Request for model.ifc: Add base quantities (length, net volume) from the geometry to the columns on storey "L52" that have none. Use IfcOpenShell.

First a look at what the model holds.

```python
import ifcopenshell
import ifcopenshell.util.element
import ifcopenshell.util.unit

model = ifcopenshell.open("model.ifc")
print(model.schema)
for unit_type in ("LENGTHUNIT", "AREAUNIT", "VOLUMEUNIT"):
    print(unit_type, ifcopenshell.util.unit.calculate_unit_scale(model, unit_type))
storey = next(s for s in model.by_type("IfcBuildingStorey") if s.Name == "L52")
columns = [e for e in ifcopenshell.util.element.get_decomposition(storey) if e.is_a("IfcColumn")]
for e in sorted(columns, key=lambda e: e.id()):
    print(e.id(), e.is_a(), e.Name, list(ifcopenshell.util.element.get_psets(e, qtos_only=True)), sep=" | ")
```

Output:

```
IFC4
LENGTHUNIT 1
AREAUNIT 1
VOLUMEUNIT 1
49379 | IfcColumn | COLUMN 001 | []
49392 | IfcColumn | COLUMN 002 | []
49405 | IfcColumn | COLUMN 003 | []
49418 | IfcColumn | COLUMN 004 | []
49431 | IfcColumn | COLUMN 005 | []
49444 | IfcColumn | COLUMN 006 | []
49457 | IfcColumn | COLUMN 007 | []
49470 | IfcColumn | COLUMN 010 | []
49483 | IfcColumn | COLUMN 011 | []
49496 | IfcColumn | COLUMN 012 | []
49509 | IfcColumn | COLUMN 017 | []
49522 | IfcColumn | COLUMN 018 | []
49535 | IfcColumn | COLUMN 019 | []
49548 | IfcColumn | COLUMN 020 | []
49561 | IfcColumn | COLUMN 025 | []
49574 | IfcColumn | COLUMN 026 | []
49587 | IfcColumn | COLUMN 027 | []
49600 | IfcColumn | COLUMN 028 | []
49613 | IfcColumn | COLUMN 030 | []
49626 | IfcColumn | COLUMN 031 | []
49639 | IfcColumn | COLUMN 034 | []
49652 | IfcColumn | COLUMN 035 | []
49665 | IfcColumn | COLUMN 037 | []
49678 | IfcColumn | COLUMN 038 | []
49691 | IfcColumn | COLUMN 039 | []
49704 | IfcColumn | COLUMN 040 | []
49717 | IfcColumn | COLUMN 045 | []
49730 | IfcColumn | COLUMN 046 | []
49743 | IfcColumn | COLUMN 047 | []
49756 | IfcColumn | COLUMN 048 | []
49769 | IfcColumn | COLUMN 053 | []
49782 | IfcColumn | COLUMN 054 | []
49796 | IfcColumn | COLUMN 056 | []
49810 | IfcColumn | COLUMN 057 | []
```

```python
import ifcopenshell
import ifcopenshell.api.pset
import ifcopenshell.geom
import ifcopenshell.util.element
import ifcopenshell.util.shape
import ifcopenshell.util.unit

model = ifcopenshell.open("model.ifc")
unit_scale = ifcopenshell.util.unit.calculate_unit_scale(model)
volume_scale = ifcopenshell.util.unit.calculate_unit_scale(model, "VOLUMEUNIT")
settings = ifcopenshell.geom.settings()

storey = next(s for s in model.by_type("IfcBuildingStorey") if s.Name == "L52")
columns = [e for e in ifcopenshell.util.element.get_decomposition(storey) if e.is_a("IfcColumn")]

for e in sorted(columns, key=lambda e: e.id()):
    if ifcopenshell.util.element.get_psets(e, qtos_only=True, should_inherit=False):
        continue
    # Geometry comes back in metres, in the element's own axes.
    shape = ifcopenshell.geom.create_shape(settings, e)
    values = {
        "Length": ifcopenshell.util.shape.get_z(shape.geometry) / unit_scale,
        "NetVolume": ifcopenshell.util.shape.get_volume(shape.geometry) / volume_scale,
    }
    qto = ifcopenshell.api.pset.add_qto(model, product=e, name="Qto_ColumnBaseQuantities")
    ifcopenshell.api.pset.edit_qto(model, qto=qto, properties=values)
    print(e.id(), {k: round(v, 3) for k, v in values.items()})

model.write("model-out.ifc")
```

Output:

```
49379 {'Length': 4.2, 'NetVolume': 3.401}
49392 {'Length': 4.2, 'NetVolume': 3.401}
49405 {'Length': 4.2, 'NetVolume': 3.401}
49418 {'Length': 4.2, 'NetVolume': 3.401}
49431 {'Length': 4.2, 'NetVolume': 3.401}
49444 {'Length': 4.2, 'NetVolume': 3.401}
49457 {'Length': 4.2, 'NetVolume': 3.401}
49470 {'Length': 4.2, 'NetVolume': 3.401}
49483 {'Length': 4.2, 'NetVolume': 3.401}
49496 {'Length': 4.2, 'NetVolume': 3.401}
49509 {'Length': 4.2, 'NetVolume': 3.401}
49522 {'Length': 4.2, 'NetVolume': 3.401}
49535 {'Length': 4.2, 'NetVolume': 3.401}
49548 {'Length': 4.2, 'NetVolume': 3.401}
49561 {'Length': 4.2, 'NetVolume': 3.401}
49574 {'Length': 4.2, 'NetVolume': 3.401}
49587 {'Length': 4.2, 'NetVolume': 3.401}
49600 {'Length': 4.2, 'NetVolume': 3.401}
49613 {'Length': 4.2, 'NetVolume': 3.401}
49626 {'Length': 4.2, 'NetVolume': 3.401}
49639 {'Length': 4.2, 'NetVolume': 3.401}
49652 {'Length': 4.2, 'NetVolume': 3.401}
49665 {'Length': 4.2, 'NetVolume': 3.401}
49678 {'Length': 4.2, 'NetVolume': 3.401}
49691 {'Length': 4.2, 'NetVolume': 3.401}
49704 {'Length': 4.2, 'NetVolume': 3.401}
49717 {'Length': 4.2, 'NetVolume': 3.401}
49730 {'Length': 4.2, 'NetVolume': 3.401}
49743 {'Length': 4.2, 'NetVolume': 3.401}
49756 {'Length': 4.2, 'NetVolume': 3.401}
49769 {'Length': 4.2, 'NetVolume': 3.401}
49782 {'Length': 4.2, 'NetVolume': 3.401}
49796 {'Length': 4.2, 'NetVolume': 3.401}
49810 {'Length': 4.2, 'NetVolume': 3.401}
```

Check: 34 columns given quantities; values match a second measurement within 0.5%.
